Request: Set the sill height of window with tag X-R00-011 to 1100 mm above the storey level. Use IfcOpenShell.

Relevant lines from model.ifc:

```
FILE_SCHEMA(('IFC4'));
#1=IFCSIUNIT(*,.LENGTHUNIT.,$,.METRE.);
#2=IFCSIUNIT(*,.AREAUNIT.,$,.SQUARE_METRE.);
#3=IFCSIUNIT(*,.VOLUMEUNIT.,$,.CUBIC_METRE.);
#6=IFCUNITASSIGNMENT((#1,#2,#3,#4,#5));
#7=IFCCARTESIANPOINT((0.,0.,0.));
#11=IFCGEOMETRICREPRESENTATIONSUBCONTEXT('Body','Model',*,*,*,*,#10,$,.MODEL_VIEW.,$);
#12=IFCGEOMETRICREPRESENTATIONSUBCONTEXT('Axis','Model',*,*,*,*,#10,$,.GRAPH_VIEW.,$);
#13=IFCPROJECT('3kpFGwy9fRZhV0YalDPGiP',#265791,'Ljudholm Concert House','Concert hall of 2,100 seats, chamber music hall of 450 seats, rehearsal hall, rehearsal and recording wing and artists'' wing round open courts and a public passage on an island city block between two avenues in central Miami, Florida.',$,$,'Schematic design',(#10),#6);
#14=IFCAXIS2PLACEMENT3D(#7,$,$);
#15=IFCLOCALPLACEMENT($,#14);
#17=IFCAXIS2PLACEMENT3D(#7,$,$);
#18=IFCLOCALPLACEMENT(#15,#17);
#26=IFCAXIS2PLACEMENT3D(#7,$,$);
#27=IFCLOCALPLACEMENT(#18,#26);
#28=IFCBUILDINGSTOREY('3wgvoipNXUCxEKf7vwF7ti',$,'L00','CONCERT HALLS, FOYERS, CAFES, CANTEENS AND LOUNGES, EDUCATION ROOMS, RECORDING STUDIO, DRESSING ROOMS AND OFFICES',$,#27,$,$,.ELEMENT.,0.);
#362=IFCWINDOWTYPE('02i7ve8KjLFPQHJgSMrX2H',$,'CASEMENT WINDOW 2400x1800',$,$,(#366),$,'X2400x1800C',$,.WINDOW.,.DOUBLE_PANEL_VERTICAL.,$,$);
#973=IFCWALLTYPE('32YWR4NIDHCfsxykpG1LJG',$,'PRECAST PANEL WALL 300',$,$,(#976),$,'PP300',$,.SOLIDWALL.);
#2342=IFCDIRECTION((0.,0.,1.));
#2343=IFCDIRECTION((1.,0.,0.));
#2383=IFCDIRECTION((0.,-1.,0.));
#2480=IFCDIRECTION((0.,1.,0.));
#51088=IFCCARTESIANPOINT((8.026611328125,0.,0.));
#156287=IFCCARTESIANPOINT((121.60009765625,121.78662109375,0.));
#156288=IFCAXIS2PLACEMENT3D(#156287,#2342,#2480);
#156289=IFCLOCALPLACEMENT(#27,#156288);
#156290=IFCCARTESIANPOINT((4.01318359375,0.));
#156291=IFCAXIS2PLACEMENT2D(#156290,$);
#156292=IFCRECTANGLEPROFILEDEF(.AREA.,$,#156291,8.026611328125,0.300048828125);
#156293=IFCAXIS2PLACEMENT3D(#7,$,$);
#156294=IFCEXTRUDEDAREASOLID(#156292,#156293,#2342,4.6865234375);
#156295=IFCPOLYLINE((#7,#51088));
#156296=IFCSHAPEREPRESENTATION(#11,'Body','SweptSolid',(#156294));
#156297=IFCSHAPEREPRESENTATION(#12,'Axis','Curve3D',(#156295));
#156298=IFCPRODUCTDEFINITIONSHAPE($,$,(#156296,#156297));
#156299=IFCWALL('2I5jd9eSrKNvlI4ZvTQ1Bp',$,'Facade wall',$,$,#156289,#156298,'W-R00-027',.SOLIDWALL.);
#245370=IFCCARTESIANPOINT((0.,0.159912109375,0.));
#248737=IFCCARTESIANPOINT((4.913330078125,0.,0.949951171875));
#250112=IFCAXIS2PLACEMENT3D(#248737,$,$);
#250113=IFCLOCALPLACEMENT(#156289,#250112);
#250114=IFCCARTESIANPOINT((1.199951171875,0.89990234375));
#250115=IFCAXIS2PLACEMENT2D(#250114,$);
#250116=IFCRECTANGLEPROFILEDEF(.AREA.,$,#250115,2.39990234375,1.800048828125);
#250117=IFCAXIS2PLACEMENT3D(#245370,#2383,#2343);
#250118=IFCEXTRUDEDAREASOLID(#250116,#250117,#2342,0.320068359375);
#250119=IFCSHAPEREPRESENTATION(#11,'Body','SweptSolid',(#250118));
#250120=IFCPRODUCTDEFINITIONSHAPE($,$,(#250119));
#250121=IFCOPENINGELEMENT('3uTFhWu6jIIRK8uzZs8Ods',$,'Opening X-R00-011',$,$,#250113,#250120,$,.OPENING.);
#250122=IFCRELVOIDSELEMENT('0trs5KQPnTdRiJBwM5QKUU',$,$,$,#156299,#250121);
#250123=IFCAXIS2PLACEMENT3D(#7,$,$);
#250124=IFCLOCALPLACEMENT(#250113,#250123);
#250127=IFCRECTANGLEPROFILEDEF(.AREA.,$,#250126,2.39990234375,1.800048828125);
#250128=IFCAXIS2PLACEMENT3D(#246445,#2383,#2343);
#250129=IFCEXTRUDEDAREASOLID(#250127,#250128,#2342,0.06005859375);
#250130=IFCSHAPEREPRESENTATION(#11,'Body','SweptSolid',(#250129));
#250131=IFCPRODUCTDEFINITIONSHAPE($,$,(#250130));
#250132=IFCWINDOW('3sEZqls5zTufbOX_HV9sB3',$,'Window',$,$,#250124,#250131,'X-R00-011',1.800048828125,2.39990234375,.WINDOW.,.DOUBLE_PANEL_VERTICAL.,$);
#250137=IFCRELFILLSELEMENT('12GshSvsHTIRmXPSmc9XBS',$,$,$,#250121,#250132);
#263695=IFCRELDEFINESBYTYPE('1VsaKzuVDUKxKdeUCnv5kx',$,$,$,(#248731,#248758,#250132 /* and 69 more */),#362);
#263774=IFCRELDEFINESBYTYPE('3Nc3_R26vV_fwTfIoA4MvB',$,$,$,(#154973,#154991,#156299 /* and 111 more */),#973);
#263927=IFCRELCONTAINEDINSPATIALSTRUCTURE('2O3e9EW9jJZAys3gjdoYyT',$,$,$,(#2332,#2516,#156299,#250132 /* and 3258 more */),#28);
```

```python
import numpy as np
import ifcopenshell
import ifcopenshell.api.geometry
import ifcopenshell.geom
import ifcopenshell.util.element
import ifcopenshell.util.placement
import ifcopenshell.util.shape
import ifcopenshell.util.unit

model = ifcopenshell.open("model.ifc")
unit_scale = ifcopenshell.util.unit.calculate_unit_scale(model)

window = model.by_id(250132)
opening = window.FillsVoids[0].RelatingOpeningElement
storey = ifcopenshell.util.element.get_container(window, ifc_class="IfcBuildingStorey")
level = ifcopenshell.util.placement.get_local_placement(storey.ObjectPlacement)[2, 3]

# The opening's origin need not be at the sill, so measure its lowest point.
shape = ifcopenshell.geom.create_shape(ifcopenshell.geom.settings(), opening)
bottom = ifcopenshell.util.shape.get_shape_bottom_elevation(shape, shape.geometry) / unit_scale
dz = level + 1.1 / unit_scale - bottom

shift = np.array([0.0, 0.0, dz])
# The window is placed relative to its opening, so it follows when the opening moves.
matrix = ifcopenshell.util.placement.get_local_placement(opening.ObjectPlacement)
matrix[:3, 3] += shift
ifcopenshell.api.geometry.edit_object_placement(
    model, product=opening, matrix=matrix, is_si=False, should_transform_children=True
)

print(f"moved by {dz * unit_scale:+.3f} m")

model.write("model_v2.ifc")
```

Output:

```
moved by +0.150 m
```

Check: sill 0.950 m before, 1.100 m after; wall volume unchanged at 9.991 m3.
